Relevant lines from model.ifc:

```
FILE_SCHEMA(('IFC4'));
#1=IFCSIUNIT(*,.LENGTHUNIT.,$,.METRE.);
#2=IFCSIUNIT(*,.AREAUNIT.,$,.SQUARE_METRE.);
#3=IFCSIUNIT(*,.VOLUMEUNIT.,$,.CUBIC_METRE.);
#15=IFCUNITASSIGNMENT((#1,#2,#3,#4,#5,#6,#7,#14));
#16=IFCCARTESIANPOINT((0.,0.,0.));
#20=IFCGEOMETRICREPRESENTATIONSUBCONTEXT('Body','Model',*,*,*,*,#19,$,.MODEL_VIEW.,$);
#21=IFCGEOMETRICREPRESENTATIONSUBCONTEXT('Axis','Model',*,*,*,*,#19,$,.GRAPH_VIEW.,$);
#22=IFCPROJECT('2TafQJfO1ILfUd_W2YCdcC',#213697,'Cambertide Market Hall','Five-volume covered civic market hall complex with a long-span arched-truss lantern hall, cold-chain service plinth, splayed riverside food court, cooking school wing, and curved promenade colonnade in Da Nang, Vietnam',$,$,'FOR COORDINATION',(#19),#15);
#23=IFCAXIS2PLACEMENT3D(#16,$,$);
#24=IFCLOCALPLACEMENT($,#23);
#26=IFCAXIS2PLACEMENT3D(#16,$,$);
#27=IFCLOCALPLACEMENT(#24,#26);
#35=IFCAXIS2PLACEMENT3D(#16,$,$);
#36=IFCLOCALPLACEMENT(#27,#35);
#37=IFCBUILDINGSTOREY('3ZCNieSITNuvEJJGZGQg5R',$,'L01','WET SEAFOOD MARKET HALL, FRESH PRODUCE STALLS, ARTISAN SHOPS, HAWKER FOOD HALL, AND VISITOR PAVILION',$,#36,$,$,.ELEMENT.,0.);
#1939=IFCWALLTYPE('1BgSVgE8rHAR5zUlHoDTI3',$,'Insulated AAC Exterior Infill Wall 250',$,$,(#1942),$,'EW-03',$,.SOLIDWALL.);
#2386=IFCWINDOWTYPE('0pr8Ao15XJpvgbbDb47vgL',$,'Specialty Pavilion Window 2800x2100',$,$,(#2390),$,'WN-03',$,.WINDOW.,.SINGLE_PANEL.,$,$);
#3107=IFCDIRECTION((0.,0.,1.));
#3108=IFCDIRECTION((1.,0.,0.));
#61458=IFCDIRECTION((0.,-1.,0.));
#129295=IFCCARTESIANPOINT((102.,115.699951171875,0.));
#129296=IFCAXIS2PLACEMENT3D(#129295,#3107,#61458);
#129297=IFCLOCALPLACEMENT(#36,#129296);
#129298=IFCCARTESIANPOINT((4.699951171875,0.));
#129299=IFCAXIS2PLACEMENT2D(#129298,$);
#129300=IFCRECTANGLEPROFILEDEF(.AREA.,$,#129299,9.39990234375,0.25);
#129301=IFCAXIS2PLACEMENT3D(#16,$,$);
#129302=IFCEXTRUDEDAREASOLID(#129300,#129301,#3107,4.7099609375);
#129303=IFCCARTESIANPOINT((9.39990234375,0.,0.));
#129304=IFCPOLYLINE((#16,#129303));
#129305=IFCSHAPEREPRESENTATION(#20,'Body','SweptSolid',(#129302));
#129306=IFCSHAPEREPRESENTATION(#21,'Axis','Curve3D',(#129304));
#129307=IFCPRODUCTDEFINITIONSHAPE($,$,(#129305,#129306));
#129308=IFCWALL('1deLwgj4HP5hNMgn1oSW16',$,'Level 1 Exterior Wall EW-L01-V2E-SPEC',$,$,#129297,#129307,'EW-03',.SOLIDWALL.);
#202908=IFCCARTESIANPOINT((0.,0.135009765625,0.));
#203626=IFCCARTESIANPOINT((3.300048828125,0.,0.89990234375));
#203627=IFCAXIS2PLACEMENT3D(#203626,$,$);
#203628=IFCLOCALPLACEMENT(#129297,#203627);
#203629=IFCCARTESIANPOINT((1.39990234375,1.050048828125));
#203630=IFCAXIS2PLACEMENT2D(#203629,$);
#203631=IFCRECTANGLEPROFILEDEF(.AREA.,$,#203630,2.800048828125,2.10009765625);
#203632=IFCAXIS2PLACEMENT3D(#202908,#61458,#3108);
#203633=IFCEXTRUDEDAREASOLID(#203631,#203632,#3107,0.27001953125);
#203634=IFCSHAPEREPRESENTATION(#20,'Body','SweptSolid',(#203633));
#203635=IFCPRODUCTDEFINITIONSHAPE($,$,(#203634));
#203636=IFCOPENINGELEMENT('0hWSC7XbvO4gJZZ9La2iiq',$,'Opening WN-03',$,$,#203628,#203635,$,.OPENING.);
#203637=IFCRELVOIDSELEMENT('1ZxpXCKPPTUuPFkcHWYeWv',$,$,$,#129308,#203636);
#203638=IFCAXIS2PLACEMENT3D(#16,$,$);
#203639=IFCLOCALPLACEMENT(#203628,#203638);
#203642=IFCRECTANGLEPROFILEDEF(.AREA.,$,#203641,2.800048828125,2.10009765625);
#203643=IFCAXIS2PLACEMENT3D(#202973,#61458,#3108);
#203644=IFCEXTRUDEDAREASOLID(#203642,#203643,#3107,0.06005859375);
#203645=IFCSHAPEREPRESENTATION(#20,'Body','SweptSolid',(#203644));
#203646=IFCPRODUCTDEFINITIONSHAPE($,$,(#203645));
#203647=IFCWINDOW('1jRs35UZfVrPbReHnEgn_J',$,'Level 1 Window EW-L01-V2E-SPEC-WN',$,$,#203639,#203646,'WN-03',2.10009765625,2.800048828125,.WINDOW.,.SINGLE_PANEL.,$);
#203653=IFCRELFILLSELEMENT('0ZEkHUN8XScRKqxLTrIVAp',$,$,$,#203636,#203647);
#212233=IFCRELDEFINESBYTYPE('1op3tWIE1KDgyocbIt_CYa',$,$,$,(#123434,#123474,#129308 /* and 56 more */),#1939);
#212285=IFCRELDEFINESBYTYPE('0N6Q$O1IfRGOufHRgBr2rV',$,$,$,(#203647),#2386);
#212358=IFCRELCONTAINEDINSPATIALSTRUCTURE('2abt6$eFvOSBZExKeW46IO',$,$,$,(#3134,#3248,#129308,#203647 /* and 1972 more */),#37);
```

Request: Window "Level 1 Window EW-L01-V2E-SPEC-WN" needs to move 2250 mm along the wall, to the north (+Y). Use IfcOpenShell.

```python
import ifcopenshell
import ifcopenshell.api.geometry
import ifcopenshell.util.placement
import ifcopenshell.util.unit

model = ifcopenshell.open("model.ifc")
unit_scale = ifcopenshell.util.unit.calculate_unit_scale(model)

window = model.by_id(203647)
opening = window.FillsVoids[0].RelatingOpeningElement
wall = opening.VoidsElements[0].RelatingBuildingElement

wall_matrix = ifcopenshell.util.placement.get_local_placement(wall.ObjectPlacement)
shift = wall_matrix[:3, 0] * -2.25 / unit_scale
before = ifcopenshell.util.placement.get_local_placement(window.ObjectPlacement)[:3, 3].copy()

# The window is placed relative to its opening, so it follows when the opening moves.
matrix = ifcopenshell.util.placement.get_local_placement(opening.ObjectPlacement)
matrix[:3, 3] += shift
ifcopenshell.api.geometry.edit_object_placement(
    model, product=opening, matrix=matrix, is_si=False, should_transform_children=True
)

after = ifcopenshell.util.placement.get_local_placement(window.ObjectPlacement)[:3, 3]
print("window moved by", (after - before).round(3) + 0.0)

model.write("model-out.ifc")
```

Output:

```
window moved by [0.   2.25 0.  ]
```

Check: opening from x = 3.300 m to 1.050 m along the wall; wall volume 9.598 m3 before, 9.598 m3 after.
